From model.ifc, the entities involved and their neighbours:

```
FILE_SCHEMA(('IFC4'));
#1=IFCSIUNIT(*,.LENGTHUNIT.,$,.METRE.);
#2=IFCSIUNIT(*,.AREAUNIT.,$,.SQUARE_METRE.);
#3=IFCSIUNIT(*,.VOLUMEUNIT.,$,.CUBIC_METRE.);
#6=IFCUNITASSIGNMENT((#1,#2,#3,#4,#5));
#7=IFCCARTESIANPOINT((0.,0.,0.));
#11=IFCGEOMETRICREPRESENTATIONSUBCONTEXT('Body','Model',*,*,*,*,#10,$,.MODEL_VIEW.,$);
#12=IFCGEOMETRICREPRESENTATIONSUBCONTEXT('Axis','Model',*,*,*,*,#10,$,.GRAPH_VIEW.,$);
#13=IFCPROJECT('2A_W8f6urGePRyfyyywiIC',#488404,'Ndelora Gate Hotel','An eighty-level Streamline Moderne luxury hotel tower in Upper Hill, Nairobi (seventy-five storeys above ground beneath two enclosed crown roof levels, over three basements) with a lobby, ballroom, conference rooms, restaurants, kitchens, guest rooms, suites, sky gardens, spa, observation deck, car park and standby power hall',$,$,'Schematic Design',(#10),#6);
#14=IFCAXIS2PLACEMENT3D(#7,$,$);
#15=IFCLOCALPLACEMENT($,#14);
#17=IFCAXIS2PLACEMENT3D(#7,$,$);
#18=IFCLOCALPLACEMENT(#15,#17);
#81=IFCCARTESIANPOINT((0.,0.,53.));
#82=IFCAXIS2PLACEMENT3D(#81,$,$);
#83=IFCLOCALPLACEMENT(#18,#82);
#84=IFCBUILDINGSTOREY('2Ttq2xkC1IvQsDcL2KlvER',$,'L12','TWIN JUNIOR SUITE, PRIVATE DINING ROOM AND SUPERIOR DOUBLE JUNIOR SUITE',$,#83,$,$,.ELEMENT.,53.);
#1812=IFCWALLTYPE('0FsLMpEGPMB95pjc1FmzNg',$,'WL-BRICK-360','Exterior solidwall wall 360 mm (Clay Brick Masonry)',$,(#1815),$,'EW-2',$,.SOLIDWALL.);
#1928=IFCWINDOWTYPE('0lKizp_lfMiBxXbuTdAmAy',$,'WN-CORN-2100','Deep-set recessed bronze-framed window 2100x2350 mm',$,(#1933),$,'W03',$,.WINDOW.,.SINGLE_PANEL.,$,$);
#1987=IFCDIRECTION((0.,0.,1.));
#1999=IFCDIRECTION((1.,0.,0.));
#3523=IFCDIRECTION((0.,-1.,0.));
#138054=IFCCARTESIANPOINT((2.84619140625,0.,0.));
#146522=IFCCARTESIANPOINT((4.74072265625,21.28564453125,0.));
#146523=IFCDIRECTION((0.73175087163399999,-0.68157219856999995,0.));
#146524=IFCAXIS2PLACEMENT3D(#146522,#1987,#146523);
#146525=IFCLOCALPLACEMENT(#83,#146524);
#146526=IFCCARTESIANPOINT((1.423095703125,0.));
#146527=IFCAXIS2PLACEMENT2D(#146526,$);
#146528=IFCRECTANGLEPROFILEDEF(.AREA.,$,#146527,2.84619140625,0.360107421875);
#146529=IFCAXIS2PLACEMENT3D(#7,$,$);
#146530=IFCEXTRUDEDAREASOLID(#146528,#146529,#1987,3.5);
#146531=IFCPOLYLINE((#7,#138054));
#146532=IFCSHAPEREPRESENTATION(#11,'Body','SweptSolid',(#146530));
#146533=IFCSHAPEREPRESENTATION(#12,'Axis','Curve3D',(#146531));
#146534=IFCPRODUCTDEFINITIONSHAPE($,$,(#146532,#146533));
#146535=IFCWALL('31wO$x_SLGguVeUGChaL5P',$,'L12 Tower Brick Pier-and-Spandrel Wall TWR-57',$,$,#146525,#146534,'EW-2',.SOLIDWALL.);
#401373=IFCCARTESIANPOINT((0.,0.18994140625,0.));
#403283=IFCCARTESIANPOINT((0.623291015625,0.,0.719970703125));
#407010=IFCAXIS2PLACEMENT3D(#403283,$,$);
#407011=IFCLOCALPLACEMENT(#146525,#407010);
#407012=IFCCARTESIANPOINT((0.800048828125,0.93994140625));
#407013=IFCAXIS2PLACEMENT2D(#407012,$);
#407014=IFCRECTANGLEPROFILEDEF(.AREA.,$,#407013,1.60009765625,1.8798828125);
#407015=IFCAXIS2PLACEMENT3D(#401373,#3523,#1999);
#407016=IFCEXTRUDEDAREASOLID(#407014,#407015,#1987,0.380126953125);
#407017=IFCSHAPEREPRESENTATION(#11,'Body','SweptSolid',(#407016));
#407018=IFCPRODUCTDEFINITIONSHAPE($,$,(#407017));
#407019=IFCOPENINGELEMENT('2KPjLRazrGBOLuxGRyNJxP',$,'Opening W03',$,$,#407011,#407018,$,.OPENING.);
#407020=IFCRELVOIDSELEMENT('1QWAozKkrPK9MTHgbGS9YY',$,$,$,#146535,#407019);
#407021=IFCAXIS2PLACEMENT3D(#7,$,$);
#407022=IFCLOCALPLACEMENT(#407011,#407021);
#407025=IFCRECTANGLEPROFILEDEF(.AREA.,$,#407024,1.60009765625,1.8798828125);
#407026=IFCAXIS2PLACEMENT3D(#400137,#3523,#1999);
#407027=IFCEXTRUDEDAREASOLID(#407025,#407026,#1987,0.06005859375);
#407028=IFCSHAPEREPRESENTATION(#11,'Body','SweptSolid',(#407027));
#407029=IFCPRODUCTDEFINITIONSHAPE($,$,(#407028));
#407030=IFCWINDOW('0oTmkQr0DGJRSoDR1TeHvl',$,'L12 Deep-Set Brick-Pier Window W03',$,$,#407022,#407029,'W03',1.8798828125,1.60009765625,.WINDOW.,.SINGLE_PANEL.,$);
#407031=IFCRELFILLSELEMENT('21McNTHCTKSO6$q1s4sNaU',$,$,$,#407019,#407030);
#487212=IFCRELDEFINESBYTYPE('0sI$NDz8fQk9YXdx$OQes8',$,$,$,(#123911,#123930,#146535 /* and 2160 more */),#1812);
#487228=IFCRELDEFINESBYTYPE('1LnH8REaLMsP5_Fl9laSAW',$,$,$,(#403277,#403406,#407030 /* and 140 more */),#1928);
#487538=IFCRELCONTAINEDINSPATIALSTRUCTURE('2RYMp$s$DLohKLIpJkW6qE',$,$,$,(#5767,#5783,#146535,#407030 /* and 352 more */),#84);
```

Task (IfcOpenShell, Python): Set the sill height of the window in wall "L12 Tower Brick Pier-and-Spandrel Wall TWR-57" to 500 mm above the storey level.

```python
import numpy as np
import ifcopenshell
import ifcopenshell.api.geometry
import ifcopenshell.geom
import ifcopenshell.util.element
import ifcopenshell.util.placement
import ifcopenshell.util.shape
import ifcopenshell.util.unit

model = ifcopenshell.open("model.ifc")
unit_scale = ifcopenshell.util.unit.calculate_unit_scale(model)

window = model.by_guid("0oTmkQr0DGJRSoDR1TeHvl")
opening = window.FillsVoids[0].RelatingOpeningElement
storey = ifcopenshell.util.element.get_container(window, ifc_class="IfcBuildingStorey")
level = ifcopenshell.util.placement.get_local_placement(storey.ObjectPlacement)[2, 3]

# The opening's origin need not be at the sill, so measure its lowest point.
shape = ifcopenshell.geom.create_shape(ifcopenshell.geom.settings(), opening)
bottom = ifcopenshell.util.shape.get_shape_bottom_elevation(shape, shape.geometry) / unit_scale
dz = level + 0.5 / unit_scale - bottom

shift = np.array([0.0, 0.0, dz])
# The window is placed relative to its opening, so it follows when the opening moves.
matrix = ifcopenshell.util.placement.get_local_placement(opening.ObjectPlacement)
matrix[:3, 3] += shift
ifcopenshell.api.geometry.edit_object_placement(
    model, product=opening, matrix=matrix, is_si=False, should_transform_children=True
)

print(f"moved by {dz * unit_scale:+.3f} m")

model.write("model_v2.ifc")
```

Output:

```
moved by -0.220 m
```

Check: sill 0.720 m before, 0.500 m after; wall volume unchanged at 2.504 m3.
